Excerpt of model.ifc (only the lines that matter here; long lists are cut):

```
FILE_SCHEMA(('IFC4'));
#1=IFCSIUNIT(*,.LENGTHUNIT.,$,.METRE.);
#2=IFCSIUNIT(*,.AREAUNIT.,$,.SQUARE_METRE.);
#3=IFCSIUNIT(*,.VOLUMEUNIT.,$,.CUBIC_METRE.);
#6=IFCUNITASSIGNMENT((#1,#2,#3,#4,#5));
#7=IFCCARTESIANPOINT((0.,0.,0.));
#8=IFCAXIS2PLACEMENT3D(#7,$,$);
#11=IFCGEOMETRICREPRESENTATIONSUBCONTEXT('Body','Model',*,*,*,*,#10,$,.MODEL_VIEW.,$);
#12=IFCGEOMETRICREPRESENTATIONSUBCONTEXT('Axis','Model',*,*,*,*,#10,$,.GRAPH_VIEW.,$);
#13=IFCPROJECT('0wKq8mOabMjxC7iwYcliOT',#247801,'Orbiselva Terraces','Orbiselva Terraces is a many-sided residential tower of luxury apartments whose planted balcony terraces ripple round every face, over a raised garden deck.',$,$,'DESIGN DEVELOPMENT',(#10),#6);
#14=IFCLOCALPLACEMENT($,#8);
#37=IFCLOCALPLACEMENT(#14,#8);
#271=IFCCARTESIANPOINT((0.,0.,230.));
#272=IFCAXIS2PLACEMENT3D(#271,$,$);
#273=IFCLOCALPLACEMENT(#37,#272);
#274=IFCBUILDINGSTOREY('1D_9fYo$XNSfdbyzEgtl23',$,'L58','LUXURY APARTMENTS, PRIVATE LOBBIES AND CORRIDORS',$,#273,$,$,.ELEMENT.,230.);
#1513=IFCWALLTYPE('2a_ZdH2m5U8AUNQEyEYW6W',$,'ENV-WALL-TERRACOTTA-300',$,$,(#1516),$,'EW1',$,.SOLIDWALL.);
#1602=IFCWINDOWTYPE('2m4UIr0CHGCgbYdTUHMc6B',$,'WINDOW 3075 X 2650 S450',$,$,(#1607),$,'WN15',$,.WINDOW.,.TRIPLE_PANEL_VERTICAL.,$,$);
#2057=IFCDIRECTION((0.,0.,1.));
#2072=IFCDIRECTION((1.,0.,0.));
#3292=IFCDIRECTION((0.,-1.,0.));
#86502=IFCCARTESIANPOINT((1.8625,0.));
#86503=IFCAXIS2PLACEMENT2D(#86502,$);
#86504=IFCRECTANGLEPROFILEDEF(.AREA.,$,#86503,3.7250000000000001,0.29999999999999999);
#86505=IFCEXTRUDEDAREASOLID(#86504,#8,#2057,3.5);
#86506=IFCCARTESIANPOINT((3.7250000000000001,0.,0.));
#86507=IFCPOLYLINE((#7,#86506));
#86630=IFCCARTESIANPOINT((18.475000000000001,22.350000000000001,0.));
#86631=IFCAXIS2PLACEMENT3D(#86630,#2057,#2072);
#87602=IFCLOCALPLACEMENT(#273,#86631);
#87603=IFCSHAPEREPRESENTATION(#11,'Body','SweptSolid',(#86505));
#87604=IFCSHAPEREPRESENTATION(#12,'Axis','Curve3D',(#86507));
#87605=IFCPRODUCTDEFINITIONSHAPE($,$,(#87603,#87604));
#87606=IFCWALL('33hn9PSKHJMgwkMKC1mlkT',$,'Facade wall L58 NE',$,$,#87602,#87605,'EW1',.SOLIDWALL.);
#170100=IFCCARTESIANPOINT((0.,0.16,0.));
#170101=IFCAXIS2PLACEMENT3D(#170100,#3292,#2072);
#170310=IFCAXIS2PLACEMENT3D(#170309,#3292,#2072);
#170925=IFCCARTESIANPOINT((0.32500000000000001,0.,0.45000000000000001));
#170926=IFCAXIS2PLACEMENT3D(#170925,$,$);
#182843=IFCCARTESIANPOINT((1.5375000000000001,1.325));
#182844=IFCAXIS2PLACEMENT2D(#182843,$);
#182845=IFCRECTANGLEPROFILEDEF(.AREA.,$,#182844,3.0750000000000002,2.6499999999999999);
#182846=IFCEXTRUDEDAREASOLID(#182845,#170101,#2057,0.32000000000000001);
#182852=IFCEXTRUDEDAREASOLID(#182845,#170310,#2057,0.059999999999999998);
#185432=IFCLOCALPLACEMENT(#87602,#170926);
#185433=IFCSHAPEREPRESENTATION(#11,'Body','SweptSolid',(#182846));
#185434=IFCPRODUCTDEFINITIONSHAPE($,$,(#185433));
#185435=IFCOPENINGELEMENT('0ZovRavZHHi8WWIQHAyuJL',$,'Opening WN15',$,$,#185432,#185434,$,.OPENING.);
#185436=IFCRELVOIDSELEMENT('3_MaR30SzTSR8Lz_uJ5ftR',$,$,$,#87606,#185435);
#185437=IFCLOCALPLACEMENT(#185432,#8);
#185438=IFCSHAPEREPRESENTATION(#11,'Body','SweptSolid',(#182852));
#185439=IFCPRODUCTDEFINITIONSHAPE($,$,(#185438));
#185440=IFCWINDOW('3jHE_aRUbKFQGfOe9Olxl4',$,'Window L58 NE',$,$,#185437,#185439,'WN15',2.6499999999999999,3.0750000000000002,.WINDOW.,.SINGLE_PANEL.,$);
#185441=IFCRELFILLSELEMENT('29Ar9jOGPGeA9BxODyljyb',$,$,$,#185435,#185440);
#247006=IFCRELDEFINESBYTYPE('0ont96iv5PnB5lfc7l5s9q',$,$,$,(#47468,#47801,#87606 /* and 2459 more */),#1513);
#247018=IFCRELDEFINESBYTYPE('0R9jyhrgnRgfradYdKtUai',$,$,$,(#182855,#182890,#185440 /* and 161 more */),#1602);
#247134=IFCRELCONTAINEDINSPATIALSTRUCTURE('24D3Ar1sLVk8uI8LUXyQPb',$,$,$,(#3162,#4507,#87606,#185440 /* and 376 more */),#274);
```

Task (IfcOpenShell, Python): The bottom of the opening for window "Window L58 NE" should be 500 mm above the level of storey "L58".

```python
import numpy as np
import ifcopenshell
import ifcopenshell.api.geometry
import ifcopenshell.geom
import ifcopenshell.util.element
import ifcopenshell.util.placement
import ifcopenshell.util.shape
import ifcopenshell.util.unit

model = ifcopenshell.open("model.ifc")
unit_scale = ifcopenshell.util.unit.calculate_unit_scale(model)

window = model.by_id(185440)
opening = window.FillsVoids[0].RelatingOpeningElement
storey = ifcopenshell.util.element.get_container(window, ifc_class="IfcBuildingStorey")
level = ifcopenshell.util.placement.get_local_placement(storey.ObjectPlacement)[2, 3]

# The opening's origin need not be at the sill, so measure its lowest point.
shape = ifcopenshell.geom.create_shape(ifcopenshell.geom.settings(), opening)
bottom = ifcopenshell.util.shape.get_shape_bottom_elevation(shape, shape.geometry) / unit_scale
dz = level + 0.5 / unit_scale - bottom

shift = np.array([0.0, 0.0, dz])
# The window is placed relative to its opening, so it follows when the opening moves.
matrix = ifcopenshell.util.placement.get_local_placement(opening.ObjectPlacement)
matrix[:3, 3] += shift
ifcopenshell.api.geometry.edit_object_placement(
    model, product=opening, matrix=matrix, is_si=False, should_transform_children=True
)

print(f"moved by {dz * unit_scale:+.3f} m")

model.write("model-out.ifc")
```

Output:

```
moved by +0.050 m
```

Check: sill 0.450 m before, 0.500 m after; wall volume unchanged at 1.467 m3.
